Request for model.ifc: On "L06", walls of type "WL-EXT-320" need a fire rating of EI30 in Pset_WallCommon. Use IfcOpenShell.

First a look at what the model holds.

```python
import ifcopenshell
import ifcopenshell.util.element

model = ifcopenshell.open("model.ifc")
print(model.schema)
storey = next(s for s in model.by_type("IfcBuildingStorey") if s.Name == "L06")
walls = [e for e in ifcopenshell.util.element.get_decomposition(storey) if e.is_a("IfcWall")]
seen = {}
for e in walls:
    element_type = ifcopenshell.util.element.get_type(e)
    key = (element_type.Name if element_type != e and element_type else None, ifcopenshell.util.element.get_pset(e, "Pset_WallCommon", "FireRating"))
    seen[key] = seen.get(key, 0) + 1
for (name, value), count in sorted(seen.items(), key=str):
    print(count, "x", name, "|", value)
```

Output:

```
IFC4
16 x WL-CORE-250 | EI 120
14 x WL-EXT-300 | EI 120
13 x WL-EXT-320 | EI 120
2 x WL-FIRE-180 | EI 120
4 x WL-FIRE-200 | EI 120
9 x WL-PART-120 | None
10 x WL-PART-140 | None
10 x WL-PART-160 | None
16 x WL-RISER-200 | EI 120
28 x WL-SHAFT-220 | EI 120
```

```python
import ifcopenshell
import ifcopenshell.api.pset
import ifcopenshell.util.element

model = ifcopenshell.open("model.ifc")

storey = next(s for s in model.by_type("IfcBuildingStorey") if s.Name == "L06")
walls = [e for e in ifcopenshell.util.element.get_decomposition(storey) if e.is_a("IfcWall")]

count = 0
for e in walls:
    element_type = ifcopenshell.util.element.get_type(e)
    if element_type in (None, e) or element_type.Name != "WL-EXT-320":
        continue
    # add_pset returns the element's existing set when there is one.
    pset = ifcopenshell.api.pset.add_pset(model, product=e, name="Pset_WallCommon")
    ifcopenshell.api.pset.edit_pset(model, pset=pset, properties={"FireRating": "EI30"})
    count += 1

print(count, "walls updated")

model.write("model_updated.ifc")
```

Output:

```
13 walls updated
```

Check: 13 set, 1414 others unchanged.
